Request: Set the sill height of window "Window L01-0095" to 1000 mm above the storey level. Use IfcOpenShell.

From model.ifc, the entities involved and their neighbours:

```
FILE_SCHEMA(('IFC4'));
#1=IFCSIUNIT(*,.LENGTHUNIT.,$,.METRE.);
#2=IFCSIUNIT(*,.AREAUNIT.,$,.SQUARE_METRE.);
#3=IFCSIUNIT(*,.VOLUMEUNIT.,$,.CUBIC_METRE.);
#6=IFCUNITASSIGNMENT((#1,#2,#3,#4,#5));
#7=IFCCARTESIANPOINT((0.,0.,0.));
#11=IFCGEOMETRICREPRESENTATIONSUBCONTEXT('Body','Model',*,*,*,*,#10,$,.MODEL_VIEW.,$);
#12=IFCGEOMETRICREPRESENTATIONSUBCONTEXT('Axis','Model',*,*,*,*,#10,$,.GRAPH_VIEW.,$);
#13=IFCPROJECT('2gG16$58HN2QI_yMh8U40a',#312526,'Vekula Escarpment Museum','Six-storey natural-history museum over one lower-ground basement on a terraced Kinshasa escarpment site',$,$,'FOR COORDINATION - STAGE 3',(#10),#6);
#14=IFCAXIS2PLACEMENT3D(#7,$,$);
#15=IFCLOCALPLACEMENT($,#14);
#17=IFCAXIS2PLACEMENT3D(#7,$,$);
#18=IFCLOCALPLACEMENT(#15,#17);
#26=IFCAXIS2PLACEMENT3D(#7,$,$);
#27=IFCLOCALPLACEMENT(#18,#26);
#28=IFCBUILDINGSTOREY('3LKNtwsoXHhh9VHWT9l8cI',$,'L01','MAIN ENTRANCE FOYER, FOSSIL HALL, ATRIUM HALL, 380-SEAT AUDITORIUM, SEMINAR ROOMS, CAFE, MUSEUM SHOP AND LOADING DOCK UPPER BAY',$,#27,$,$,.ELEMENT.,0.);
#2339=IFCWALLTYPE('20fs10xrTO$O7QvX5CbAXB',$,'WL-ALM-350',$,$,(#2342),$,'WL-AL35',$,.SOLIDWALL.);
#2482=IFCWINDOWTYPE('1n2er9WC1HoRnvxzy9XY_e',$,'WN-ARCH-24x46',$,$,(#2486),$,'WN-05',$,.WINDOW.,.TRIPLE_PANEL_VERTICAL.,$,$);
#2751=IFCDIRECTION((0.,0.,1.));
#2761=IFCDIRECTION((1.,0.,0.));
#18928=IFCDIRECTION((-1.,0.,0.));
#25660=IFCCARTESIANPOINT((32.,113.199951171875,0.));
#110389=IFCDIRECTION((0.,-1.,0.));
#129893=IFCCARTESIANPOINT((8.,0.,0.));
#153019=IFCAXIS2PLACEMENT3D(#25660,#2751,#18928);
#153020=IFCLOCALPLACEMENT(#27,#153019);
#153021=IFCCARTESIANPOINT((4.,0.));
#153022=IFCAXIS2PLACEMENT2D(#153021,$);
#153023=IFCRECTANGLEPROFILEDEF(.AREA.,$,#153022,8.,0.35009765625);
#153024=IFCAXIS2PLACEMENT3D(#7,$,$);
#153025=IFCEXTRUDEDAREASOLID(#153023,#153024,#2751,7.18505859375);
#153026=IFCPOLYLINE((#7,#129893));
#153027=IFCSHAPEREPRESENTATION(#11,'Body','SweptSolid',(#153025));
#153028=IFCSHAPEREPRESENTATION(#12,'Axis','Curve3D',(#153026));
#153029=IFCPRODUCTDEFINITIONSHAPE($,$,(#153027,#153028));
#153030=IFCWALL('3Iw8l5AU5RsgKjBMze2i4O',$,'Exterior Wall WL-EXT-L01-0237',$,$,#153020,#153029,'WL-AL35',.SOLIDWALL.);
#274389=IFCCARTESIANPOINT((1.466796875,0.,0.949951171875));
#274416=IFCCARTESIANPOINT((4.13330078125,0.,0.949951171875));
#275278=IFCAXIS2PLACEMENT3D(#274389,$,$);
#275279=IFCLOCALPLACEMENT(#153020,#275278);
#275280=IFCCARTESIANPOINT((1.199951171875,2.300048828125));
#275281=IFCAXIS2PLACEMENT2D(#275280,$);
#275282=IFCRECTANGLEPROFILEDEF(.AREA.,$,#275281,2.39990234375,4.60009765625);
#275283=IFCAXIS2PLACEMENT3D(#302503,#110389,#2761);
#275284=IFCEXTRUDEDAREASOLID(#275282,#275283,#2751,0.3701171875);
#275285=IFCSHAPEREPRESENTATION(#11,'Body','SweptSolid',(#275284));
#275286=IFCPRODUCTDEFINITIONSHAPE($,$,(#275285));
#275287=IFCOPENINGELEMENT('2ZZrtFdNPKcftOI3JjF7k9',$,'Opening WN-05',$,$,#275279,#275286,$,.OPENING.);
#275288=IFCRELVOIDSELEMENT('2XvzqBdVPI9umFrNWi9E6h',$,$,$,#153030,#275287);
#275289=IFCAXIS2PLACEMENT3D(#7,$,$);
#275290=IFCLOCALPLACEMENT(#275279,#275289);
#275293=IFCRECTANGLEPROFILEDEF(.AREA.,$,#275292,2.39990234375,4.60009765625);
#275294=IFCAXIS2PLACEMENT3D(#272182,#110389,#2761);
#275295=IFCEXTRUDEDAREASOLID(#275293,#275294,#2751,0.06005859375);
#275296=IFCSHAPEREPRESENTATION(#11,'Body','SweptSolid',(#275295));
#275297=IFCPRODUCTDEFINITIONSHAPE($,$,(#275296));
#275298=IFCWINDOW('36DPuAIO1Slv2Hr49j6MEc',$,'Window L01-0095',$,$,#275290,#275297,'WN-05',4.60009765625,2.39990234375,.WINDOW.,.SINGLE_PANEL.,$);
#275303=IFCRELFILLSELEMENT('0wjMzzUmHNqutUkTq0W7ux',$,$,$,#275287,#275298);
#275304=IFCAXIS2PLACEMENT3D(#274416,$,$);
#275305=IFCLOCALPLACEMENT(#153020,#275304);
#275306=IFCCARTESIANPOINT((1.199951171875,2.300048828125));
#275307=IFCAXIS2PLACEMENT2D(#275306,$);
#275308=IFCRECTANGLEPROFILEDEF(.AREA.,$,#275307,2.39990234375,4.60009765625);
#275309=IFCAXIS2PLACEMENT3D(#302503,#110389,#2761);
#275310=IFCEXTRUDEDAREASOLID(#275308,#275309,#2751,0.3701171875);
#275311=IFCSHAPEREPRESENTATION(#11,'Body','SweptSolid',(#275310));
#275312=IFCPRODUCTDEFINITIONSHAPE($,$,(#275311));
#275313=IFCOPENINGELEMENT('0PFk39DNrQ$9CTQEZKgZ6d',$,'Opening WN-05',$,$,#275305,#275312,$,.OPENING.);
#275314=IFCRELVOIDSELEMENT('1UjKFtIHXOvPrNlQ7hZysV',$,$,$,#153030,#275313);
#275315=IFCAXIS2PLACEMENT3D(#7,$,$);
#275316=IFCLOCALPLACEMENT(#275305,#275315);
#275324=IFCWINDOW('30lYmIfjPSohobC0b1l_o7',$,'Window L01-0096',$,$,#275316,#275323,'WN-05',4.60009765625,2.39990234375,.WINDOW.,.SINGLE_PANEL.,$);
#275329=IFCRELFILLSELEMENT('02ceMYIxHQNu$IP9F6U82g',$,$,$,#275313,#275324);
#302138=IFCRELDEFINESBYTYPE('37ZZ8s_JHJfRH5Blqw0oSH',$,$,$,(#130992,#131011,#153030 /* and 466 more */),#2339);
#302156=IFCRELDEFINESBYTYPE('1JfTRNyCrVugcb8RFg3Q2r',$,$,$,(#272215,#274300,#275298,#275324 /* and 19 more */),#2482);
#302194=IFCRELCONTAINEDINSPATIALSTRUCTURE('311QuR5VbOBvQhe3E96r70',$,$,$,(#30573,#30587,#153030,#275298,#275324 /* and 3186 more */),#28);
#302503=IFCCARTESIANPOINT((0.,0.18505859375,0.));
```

```python
import numpy as np
import ifcopenshell
import ifcopenshell.api.geometry
import ifcopenshell.geom
import ifcopenshell.util.element
import ifcopenshell.util.placement
import ifcopenshell.util.shape
import ifcopenshell.util.unit

model = ifcopenshell.open("model.ifc")
unit_scale = ifcopenshell.util.unit.calculate_unit_scale(model)

window = model.by_guid("36DPuAIO1Slv2Hr49j6MEc")
opening = window.FillsVoids[0].RelatingOpeningElement
storey = ifcopenshell.util.element.get_container(window, ifc_class="IfcBuildingStorey")
level = ifcopenshell.util.placement.get_local_placement(storey.ObjectPlacement)[2, 3]

# The opening's origin need not be at the sill, so measure its lowest point.
shape = ifcopenshell.geom.create_shape(ifcopenshell.geom.settings(), opening)
bottom = ifcopenshell.util.shape.get_shape_bottom_elevation(shape, shape.geometry) / unit_scale
dz = level + 1 / unit_scale - bottom

shift = np.array([0.0, 0.0, dz])
# The window is placed relative to its opening, so it follows when the opening moves.
matrix = ifcopenshell.util.placement.get_local_placement(opening.ObjectPlacement)
matrix[:3, 3] += shift
ifcopenshell.api.geometry.edit_object_placement(
    model, product=opening, matrix=matrix, is_si=False, should_transform_children=True
)

print(f"moved by {dz * unit_scale:+.3f} m")

model.write("model_updated.ifc")
```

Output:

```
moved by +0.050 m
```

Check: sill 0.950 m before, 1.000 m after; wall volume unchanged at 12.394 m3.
